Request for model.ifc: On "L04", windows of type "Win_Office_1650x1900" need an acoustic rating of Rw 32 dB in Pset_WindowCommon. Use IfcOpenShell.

First a look at what the model holds.

```python
import ifcopenshell
import ifcopenshell.util.element

model = ifcopenshell.open("model.ifc")
print(model.schema)
storey = next(s for s in model.by_type("IfcBuildingStorey") if s.Name == "L04")
windows = [e for e in ifcopenshell.util.element.get_decomposition(storey) if e.is_a("IfcWindow")]
seen = {}
for e in windows:
    element_type = ifcopenshell.util.element.get_type(e)
    key = (element_type.Name if element_type != e and element_type else None, ifcopenshell.util.element.get_pset(e, "Pset_WindowCommon", "AcousticRating"))
    seen[key] = seen.get(key, 0) + 1
for (name, value), count in sorted(seen.items(), key=str):
    print(count, "x", name, "|", value)
```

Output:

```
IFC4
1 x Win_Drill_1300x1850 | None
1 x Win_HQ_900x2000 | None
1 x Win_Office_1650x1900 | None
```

```python
import ifcopenshell
import ifcopenshell.api.pset
import ifcopenshell.util.element

model = ifcopenshell.open("model.ifc")

storey = next(s for s in model.by_type("IfcBuildingStorey") if s.Name == "L04")
windows = [e for e in ifcopenshell.util.element.get_decomposition(storey) if e.is_a("IfcWindow")]

count = 0
for e in windows:
    element_type = ifcopenshell.util.element.get_type(e)
    if element_type in (None, e) or element_type.Name != "Win_Office_1650x1900":
        continue
    # add_pset returns the element's existing set when there is one.
    pset = ifcopenshell.api.pset.add_pset(model, product=e, name="Pset_WindowCommon")
    ifcopenshell.api.pset.edit_pset(model, pset=pset, properties={"AcousticRating": "Rw 32 dB"})
    count += 1

print(count, "windows updated")

model.write("model_rev.ifc")
```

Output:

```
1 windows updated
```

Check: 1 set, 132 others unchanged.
